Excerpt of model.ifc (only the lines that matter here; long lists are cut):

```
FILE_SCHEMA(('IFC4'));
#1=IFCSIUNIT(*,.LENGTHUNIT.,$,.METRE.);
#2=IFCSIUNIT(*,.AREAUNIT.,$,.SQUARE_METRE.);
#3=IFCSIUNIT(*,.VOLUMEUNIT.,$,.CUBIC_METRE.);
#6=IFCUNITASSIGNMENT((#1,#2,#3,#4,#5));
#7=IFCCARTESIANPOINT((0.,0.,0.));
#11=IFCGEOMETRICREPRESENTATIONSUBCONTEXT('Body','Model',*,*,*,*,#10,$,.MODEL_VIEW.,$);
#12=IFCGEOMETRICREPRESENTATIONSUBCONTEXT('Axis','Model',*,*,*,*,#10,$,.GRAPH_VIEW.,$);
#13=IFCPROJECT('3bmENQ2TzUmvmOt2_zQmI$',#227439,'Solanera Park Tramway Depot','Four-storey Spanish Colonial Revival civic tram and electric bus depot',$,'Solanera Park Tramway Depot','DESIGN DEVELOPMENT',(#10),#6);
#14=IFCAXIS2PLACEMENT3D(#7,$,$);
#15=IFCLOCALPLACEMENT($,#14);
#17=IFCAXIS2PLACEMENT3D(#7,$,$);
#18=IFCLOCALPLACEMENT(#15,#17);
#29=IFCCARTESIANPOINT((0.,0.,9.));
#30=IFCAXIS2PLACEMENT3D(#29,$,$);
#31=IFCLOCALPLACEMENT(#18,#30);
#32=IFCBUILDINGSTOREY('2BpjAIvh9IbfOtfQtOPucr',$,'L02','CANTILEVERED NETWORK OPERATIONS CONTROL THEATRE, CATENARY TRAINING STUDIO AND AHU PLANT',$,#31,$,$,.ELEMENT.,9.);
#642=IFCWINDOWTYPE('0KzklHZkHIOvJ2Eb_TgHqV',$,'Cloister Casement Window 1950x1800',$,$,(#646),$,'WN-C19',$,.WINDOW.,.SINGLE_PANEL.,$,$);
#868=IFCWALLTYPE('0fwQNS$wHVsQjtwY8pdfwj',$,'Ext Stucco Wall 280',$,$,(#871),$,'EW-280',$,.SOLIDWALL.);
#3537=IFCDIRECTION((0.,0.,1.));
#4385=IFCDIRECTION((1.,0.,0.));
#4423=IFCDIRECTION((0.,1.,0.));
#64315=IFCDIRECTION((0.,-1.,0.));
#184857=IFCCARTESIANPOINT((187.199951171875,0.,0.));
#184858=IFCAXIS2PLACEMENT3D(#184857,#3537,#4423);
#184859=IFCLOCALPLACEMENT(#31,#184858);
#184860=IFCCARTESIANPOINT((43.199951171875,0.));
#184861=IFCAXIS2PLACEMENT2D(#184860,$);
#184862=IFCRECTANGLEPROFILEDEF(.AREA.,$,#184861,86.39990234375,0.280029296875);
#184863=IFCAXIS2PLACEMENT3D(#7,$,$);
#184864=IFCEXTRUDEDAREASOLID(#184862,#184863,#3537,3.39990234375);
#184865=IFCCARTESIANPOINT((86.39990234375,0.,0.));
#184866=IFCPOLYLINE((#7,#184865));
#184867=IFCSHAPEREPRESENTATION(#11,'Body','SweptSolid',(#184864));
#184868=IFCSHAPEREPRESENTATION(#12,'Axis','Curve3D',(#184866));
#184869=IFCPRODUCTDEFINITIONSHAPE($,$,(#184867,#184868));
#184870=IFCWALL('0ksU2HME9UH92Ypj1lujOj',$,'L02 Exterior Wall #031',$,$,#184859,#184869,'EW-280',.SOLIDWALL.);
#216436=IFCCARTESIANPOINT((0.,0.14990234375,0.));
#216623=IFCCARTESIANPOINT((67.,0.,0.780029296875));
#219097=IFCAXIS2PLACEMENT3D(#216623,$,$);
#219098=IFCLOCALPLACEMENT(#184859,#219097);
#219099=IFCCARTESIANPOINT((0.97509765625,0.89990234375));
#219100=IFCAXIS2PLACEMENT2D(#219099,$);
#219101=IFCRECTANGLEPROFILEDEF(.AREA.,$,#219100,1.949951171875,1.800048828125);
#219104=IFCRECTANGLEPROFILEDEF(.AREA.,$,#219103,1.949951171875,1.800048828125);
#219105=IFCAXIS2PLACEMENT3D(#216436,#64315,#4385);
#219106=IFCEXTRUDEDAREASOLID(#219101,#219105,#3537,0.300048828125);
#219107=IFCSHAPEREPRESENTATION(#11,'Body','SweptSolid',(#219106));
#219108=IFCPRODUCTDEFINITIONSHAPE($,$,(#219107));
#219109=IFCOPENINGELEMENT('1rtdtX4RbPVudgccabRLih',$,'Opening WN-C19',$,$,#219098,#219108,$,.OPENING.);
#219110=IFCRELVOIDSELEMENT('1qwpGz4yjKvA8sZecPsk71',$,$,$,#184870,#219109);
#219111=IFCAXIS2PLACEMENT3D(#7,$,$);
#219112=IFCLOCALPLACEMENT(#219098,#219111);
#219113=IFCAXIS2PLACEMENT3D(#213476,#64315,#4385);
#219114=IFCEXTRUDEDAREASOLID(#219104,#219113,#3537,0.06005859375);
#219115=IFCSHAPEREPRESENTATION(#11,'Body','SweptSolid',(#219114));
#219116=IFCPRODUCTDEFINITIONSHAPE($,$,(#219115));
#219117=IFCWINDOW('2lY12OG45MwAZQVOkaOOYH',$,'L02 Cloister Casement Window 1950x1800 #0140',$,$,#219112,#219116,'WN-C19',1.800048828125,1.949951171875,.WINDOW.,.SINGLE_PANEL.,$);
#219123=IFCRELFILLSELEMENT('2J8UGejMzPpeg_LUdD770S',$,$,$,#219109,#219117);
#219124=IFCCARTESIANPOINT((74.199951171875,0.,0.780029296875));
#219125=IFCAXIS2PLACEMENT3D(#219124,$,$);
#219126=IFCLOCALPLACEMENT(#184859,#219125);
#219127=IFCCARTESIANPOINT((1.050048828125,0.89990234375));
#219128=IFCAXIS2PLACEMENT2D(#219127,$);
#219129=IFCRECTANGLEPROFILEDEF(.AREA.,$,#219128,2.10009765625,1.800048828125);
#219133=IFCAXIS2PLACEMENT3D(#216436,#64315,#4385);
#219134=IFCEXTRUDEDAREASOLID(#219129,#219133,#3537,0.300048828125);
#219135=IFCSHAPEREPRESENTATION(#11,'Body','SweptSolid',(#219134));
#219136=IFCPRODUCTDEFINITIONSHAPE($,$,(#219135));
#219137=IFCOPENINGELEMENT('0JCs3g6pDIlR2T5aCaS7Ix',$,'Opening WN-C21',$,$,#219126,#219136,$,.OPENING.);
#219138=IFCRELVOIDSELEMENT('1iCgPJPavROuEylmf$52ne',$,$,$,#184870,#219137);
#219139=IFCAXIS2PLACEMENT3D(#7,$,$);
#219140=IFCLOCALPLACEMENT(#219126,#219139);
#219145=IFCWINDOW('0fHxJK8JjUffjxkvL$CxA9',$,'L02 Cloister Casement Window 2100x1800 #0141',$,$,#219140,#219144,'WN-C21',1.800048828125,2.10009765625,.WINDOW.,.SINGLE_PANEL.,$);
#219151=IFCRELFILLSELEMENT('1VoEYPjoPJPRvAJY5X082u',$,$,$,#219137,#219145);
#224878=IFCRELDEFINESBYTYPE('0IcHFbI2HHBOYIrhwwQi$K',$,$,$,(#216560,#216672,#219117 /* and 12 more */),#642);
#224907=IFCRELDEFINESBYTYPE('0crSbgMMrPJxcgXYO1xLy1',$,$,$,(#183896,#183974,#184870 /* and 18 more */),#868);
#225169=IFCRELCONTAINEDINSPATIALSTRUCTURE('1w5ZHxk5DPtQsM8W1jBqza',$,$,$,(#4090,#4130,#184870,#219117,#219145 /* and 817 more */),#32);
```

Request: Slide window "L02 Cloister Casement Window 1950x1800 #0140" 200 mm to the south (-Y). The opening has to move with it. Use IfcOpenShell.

```python
import ifcopenshell
import ifcopenshell.api.geometry
import ifcopenshell.util.placement
import ifcopenshell.util.unit

model = ifcopenshell.open("model.ifc")
unit_scale = ifcopenshell.util.unit.calculate_unit_scale(model)

window = model.by_guid("2lY12OG45MwAZQVOkaOOYH")
opening = window.FillsVoids[0].RelatingOpeningElement
wall = opening.VoidsElements[0].RelatingBuildingElement

wall_matrix = ifcopenshell.util.placement.get_local_placement(wall.ObjectPlacement)
shift = wall_matrix[:3, 0] * -0.2 / unit_scale
before = ifcopenshell.util.placement.get_local_placement(window.ObjectPlacement)[:3, 3].copy()

# The window is placed relative to its opening, so it follows when the opening moves.
matrix = ifcopenshell.util.placement.get_local_placement(opening.ObjectPlacement)
matrix[:3, 3] += shift
ifcopenshell.api.geometry.edit_object_placement(
    model, product=opening, matrix=matrix, is_si=False, should_transform_children=True
)

after = ifcopenshell.util.placement.get_local_placement(window.ObjectPlacement)[:3, 3]
print("window moved by", (after - before).round(3) + 0.0)

model.write("model_rev.ifc")
```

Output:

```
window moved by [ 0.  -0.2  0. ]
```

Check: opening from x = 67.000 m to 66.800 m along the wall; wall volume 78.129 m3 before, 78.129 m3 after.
